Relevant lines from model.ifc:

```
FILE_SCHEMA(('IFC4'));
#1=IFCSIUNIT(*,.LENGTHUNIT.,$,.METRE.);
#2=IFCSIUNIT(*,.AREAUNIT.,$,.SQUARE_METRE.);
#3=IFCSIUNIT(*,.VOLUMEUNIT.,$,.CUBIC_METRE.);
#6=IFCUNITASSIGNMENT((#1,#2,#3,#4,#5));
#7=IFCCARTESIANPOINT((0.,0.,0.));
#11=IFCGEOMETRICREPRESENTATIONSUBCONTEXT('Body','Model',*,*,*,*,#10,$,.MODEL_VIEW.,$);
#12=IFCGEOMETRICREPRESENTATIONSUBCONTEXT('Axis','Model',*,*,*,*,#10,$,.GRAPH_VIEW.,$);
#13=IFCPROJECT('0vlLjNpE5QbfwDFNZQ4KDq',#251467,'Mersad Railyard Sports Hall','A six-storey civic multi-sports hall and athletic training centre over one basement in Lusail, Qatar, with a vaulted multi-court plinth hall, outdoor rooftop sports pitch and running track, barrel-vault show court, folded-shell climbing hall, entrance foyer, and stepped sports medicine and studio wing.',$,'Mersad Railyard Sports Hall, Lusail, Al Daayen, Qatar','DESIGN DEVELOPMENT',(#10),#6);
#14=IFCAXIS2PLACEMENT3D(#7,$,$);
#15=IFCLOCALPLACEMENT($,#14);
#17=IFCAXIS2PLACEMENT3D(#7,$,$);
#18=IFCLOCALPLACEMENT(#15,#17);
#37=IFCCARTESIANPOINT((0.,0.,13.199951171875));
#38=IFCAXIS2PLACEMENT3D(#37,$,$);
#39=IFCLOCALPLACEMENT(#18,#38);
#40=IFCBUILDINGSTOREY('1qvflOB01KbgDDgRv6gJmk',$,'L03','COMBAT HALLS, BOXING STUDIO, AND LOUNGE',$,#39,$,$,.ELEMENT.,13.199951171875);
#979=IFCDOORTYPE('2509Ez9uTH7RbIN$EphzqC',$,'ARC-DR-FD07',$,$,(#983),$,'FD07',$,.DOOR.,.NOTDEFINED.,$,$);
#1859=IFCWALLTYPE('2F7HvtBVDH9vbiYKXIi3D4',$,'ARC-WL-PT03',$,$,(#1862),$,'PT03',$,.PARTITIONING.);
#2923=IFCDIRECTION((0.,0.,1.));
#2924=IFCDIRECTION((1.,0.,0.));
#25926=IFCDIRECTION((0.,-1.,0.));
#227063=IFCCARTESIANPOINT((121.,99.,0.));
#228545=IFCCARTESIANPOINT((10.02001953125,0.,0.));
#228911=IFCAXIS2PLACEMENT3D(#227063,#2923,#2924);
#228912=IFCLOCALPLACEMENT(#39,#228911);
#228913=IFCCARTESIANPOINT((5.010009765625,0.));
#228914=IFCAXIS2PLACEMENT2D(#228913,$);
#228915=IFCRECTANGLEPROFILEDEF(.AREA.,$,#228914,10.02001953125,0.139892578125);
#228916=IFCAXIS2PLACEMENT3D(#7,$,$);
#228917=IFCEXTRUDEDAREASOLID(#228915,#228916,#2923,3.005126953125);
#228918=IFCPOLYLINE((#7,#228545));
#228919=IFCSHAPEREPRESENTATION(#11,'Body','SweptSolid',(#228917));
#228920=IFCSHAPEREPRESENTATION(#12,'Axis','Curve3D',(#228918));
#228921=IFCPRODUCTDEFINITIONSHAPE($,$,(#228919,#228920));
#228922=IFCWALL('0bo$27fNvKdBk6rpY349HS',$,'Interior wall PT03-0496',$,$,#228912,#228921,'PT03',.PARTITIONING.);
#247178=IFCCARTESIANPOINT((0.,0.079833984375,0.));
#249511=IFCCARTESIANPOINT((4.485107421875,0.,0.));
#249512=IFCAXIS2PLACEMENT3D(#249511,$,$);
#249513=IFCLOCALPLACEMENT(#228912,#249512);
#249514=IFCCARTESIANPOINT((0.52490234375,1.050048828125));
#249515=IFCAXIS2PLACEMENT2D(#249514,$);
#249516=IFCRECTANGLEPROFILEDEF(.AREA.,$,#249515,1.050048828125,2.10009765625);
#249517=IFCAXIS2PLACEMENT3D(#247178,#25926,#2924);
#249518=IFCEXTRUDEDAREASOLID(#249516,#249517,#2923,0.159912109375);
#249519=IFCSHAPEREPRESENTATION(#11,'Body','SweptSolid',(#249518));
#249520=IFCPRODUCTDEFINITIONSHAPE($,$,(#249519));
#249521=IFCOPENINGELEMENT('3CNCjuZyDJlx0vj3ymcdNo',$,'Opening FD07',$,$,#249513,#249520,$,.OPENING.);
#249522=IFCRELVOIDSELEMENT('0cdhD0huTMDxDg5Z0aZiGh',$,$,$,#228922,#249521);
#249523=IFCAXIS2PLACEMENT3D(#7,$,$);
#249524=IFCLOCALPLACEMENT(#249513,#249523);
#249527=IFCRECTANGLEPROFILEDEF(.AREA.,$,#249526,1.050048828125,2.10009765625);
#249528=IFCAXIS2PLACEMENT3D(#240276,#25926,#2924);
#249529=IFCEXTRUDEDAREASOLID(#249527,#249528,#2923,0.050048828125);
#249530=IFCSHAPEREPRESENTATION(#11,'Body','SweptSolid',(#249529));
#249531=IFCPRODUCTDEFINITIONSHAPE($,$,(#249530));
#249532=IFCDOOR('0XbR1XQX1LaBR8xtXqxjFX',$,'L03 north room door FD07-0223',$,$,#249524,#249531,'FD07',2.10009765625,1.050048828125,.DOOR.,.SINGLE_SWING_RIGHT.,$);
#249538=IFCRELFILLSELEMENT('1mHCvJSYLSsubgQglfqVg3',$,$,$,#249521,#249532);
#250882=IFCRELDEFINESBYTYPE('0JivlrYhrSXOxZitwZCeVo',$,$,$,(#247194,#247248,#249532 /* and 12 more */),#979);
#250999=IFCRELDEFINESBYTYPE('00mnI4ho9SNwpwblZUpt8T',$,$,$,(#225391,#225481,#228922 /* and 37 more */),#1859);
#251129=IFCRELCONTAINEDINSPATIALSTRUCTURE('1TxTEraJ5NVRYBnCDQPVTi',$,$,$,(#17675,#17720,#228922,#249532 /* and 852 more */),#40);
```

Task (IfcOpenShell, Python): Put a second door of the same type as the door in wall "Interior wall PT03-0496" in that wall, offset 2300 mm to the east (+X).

```python
import ifcopenshell
import ifcopenshell.api.feature
import ifcopenshell.api.geometry
import ifcopenshell.api.root
import ifcopenshell.geom
import ifcopenshell.util.element
import ifcopenshell.util.placement
import ifcopenshell.util.shape

model = ifcopenshell.open("model.ifc")
settings = ifcopenshell.geom.settings()


def volume(element):
    """Net volume in cubic metres, openings subtracted."""
    shape = ifcopenshell.geom.create_shape(settings, element)
    return ifcopenshell.util.shape.get_volume(shape.geometry)


door = model.by_guid("0XbR1XQX1LaBR8xtXqxjFX")
opening = door.FillsVoids[0].RelatingOpeningElement
wall = opening.VoidsElements[0].RelatingBuildingElement
before = volume(wall)
shift = ifcopenshell.util.placement.get_local_placement(wall.ObjectPlacement)[:3, 0] * 2.3

# copy_class copies the void relationship, type, container and properties, but no geometry.
new_opening = ifcopenshell.api.root.copy_class(model, product=opening)
new_opening.Representation = ifcopenshell.util.element.copy_deep(
    model, opening.Representation, exclude=["IfcGeometricRepresentationContext", "IfcRepresentationMap"]
)
new_door = ifcopenshell.api.root.copy_class(model, product=door)
new_door.Representation = ifcopenshell.util.element.copy_deep(
    model, door.Representation, exclude=["IfcGeometricRepresentationContext", "IfcRepresentationMap"]
)
new_door.Tag = None
ifcopenshell.api.feature.add_filling(model, opening=new_opening, element=new_door)

for old, new in ((opening, new_opening), (door, new_door)):
    matrix = ifcopenshell.util.placement.get_local_placement(old.ObjectPlacement)
    matrix[:3, 3] += shift
    ifcopenshell.api.geometry.edit_object_placement(model, product=new, matrix=matrix, is_si=False)

after = volume(wall)

print(f"wall volume {before:.3f} -> {after:.3f} m3")

model.write("model-out.ifc")
```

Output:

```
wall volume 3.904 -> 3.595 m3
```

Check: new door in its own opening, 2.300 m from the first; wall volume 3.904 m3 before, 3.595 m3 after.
